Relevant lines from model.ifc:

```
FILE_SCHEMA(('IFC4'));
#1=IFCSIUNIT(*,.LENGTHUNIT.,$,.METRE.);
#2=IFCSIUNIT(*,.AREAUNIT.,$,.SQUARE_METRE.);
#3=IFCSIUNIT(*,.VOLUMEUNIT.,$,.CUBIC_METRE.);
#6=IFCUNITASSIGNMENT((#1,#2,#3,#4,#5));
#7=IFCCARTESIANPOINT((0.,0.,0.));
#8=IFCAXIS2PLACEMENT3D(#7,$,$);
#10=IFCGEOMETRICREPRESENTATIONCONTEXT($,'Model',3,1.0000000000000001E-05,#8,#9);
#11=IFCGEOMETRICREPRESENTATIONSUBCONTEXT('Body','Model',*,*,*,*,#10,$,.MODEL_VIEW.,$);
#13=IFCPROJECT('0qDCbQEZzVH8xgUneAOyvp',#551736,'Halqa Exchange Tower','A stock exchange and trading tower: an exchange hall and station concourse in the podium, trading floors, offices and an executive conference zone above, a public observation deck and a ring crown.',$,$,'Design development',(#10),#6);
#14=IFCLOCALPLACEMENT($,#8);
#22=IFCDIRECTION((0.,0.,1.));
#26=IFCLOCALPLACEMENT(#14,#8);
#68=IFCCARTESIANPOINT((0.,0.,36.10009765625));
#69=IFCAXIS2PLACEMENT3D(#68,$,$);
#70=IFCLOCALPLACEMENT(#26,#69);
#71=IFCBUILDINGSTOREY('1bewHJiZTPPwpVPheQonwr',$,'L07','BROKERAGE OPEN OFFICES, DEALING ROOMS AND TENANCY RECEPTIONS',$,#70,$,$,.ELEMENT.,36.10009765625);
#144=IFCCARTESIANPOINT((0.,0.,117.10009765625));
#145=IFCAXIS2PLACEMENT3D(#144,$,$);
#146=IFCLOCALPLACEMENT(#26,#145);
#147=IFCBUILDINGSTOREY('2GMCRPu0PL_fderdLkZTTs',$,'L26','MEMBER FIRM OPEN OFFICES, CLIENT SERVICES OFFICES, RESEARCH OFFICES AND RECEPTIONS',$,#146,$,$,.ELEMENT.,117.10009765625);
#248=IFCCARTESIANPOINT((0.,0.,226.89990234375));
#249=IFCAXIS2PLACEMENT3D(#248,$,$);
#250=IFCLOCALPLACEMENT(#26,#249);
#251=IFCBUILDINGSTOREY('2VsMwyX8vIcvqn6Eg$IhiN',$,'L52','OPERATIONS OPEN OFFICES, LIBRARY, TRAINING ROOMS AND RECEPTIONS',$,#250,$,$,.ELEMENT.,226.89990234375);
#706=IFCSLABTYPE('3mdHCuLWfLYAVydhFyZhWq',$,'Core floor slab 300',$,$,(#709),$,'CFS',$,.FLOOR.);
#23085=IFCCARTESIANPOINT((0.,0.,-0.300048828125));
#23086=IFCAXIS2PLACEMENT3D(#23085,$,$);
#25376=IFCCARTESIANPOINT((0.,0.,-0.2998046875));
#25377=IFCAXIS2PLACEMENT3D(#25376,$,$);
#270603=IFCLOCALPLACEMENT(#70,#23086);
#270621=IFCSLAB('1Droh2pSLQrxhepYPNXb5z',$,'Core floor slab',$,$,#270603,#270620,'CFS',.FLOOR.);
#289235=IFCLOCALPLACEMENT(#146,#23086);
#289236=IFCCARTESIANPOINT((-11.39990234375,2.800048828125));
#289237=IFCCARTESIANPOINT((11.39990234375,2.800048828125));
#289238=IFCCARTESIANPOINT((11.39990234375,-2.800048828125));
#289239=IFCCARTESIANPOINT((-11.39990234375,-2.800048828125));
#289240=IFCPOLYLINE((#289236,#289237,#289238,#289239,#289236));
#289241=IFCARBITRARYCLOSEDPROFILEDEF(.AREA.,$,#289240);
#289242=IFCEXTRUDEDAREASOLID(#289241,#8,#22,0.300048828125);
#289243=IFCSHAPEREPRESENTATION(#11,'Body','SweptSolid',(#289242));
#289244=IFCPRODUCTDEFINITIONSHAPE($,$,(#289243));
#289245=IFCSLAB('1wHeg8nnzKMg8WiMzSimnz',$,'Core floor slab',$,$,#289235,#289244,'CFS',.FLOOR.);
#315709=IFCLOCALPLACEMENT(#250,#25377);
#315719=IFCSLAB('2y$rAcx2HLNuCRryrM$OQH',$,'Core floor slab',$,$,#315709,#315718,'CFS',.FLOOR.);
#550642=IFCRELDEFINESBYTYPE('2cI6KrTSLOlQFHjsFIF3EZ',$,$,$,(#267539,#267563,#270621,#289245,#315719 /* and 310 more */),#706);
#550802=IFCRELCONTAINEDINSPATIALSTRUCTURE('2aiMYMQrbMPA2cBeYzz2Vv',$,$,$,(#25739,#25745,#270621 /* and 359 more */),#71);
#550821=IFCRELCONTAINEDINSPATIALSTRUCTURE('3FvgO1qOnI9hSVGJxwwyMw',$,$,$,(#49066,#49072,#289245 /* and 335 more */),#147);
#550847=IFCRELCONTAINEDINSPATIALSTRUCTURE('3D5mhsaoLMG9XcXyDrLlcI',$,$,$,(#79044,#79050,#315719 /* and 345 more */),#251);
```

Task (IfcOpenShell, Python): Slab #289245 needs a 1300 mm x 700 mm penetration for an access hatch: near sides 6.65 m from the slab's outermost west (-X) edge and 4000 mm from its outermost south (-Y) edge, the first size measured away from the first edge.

```python
import numpy as np
import ifcopenshell
import ifcopenshell.api.feature
import ifcopenshell.api.geometry
import ifcopenshell.api.root
import ifcopenshell.geom
import ifcopenshell.util.placement
import ifcopenshell.util.representation
import ifcopenshell.util.shape
import ifcopenshell.util.unit

model = ifcopenshell.open("model.ifc")
unit_scale = ifcopenshell.util.unit.calculate_unit_scale(model)
settings = ifcopenshell.geom.settings()


def volume(element):
    """Net volume in cubic metres, openings subtracted."""
    shape = ifcopenshell.geom.create_shape(settings, element)
    return ifcopenshell.util.shape.get_volume(shape.geometry)


slab = model.by_guid("1wHeg8nnzKMg8WiMzSimnz")
before = volume(slab)

# Extent in the slab's own axes, in metres. The edges named are its -X and -Y sides.
slab_shape = ifcopenshell.geom.create_shape(settings, slab)
vertices = ifcopenshell.util.shape.get_vertices(slab_shape.geometry)
x_min, y_min, bottom = vertices.min(axis=0)
top = vertices[:, 2].max()

opening = ifcopenshell.api.root.create_entity(model, ifc_class="IfcOpeningElement", name="Access hatch opening", predefined_type="OPENING")
context = ifcopenshell.util.representation.get_context(model, "Model", "Body", "MODEL_VIEW")
width, depth = 1.3, 0.7
outline = [(0.0, 0.0), (width, 0.0), (width, depth), (0.0, depth), (0.0, 0.0)]
# Overshoot both faces by 50 mm so the cut is clean.
shape = ifcopenshell.api.geometry.add_slab_representation(
    model, context=context, depth=top - bottom + 0.1, polyline=outline
)
ifcopenshell.api.geometry.assign_representation(model, product=opening, representation=shape)

matrix = ifcopenshell.util.placement.get_local_placement(slab.ObjectPlacement)
matrix[:, 3] = matrix @ np.append(np.array([x_min + 6.65, y_min + 4, bottom - 0.05]) / unit_scale, 1.0)
ifcopenshell.api.geometry.edit_object_placement(model, product=opening, matrix=matrix, is_si=False)
ifcopenshell.api.feature.add_feature(model, feature=opening, element=slab)

after = volume(slab)

print(f"slab volume {before:.3f} -> {after:.3f} m3")

model.write("model-out.ifc")
```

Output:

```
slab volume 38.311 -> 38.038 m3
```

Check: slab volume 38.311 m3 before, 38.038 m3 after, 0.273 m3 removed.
